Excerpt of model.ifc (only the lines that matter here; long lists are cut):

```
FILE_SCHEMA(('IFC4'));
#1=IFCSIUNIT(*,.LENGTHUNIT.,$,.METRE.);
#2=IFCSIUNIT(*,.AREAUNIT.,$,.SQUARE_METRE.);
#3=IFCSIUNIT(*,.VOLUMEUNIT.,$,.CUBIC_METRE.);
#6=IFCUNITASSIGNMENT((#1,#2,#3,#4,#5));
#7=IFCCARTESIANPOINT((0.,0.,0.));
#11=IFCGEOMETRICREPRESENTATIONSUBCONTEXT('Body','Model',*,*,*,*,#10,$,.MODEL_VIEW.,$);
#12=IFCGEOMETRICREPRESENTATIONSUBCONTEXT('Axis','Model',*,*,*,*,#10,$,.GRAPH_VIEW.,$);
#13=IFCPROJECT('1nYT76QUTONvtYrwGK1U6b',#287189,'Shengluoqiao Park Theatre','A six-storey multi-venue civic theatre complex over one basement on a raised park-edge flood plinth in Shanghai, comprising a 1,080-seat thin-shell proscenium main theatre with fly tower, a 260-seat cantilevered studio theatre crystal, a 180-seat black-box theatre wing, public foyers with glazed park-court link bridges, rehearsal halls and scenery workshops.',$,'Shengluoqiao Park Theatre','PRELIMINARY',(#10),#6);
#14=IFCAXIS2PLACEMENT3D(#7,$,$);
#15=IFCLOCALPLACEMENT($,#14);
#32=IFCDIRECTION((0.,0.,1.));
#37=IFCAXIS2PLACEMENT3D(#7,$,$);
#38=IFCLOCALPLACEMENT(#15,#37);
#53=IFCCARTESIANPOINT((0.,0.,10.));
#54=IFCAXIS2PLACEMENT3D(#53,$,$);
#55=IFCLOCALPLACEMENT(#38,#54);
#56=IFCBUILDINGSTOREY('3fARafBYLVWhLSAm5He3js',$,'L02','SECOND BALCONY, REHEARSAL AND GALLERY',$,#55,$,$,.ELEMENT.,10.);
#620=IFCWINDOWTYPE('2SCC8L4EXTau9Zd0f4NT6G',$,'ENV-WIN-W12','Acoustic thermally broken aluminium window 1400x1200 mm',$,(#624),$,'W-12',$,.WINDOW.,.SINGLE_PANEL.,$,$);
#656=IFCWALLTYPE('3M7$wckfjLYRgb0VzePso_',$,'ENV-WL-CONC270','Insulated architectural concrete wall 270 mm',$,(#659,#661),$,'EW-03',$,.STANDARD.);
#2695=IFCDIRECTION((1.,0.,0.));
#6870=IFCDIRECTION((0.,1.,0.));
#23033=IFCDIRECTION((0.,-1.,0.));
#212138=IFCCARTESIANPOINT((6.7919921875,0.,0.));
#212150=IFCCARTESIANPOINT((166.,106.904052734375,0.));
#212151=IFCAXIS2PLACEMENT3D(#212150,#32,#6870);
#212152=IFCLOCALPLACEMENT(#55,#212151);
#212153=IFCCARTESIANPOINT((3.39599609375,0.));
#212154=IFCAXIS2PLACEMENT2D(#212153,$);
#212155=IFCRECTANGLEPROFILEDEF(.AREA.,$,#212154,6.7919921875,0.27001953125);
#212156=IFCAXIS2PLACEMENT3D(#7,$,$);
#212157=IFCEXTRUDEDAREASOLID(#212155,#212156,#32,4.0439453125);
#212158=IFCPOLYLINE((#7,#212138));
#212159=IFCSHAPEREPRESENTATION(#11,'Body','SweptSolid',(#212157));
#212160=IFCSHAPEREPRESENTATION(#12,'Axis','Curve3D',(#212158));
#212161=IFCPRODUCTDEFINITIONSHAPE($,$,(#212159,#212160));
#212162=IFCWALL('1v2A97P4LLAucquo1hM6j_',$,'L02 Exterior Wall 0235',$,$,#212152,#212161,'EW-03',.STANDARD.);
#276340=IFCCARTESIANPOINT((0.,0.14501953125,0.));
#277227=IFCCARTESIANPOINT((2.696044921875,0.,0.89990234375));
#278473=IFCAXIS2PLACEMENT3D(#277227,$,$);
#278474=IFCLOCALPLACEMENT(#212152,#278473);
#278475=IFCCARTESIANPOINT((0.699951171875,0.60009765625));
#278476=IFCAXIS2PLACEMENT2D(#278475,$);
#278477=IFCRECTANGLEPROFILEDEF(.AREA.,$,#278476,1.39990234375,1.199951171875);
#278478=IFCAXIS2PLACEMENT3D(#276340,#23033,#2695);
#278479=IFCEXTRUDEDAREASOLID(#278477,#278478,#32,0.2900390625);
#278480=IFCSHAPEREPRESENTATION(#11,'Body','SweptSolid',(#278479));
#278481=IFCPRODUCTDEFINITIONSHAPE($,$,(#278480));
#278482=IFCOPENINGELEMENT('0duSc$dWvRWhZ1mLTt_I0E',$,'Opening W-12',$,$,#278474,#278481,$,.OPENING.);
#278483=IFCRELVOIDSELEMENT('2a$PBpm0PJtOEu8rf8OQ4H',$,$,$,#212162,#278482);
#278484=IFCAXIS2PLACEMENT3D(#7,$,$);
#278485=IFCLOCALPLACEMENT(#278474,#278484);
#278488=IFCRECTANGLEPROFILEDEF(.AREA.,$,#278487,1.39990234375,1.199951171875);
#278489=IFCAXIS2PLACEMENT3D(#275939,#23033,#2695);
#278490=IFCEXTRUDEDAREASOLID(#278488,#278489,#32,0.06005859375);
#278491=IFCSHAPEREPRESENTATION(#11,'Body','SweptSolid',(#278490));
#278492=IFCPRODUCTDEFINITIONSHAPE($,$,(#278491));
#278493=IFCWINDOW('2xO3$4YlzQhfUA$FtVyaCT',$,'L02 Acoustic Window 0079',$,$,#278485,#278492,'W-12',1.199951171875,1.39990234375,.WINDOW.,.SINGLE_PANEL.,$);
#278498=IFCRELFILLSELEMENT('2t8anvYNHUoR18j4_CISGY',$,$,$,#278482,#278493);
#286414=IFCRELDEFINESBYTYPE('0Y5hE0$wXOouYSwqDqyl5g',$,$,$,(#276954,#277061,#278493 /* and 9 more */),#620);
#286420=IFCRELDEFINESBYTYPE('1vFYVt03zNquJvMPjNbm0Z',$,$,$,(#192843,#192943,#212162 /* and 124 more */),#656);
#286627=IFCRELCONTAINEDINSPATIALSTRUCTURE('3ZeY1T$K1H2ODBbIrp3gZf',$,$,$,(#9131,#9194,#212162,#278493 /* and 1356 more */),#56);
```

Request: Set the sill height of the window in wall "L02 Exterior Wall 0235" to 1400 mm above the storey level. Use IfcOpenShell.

```python
import numpy as np
import ifcopenshell
import ifcopenshell.api.geometry
import ifcopenshell.geom
import ifcopenshell.util.element
import ifcopenshell.util.placement
import ifcopenshell.util.shape
import ifcopenshell.util.unit

model = ifcopenshell.open("model.ifc")
unit_scale = ifcopenshell.util.unit.calculate_unit_scale(model)

window = model.by_guid("2xO3$4YlzQhfUA$FtVyaCT")
opening = window.FillsVoids[0].RelatingOpeningElement
storey = ifcopenshell.util.element.get_container(window, ifc_class="IfcBuildingStorey")
level = ifcopenshell.util.placement.get_local_placement(storey.ObjectPlacement)[2, 3]

# The opening's origin need not be at the sill, so measure its lowest point.
shape = ifcopenshell.geom.create_shape(ifcopenshell.geom.settings(), opening)
bottom = ifcopenshell.util.shape.get_shape_bottom_elevation(shape, shape.geometry) / unit_scale
dz = level + 1.4 / unit_scale - bottom

shift = np.array([0.0, 0.0, dz])
# The window is placed relative to its opening, so it follows when the opening moves.
matrix = ifcopenshell.util.placement.get_local_placement(opening.ObjectPlacement)
matrix[:3, 3] += shift
ifcopenshell.api.geometry.edit_object_placement(
    model, product=opening, matrix=matrix, is_si=False, should_transform_children=True
)

print(f"moved by {dz * unit_scale:+.3f} m")

model.write("model-out.ifc")
```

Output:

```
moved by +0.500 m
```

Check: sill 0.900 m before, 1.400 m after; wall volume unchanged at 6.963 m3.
